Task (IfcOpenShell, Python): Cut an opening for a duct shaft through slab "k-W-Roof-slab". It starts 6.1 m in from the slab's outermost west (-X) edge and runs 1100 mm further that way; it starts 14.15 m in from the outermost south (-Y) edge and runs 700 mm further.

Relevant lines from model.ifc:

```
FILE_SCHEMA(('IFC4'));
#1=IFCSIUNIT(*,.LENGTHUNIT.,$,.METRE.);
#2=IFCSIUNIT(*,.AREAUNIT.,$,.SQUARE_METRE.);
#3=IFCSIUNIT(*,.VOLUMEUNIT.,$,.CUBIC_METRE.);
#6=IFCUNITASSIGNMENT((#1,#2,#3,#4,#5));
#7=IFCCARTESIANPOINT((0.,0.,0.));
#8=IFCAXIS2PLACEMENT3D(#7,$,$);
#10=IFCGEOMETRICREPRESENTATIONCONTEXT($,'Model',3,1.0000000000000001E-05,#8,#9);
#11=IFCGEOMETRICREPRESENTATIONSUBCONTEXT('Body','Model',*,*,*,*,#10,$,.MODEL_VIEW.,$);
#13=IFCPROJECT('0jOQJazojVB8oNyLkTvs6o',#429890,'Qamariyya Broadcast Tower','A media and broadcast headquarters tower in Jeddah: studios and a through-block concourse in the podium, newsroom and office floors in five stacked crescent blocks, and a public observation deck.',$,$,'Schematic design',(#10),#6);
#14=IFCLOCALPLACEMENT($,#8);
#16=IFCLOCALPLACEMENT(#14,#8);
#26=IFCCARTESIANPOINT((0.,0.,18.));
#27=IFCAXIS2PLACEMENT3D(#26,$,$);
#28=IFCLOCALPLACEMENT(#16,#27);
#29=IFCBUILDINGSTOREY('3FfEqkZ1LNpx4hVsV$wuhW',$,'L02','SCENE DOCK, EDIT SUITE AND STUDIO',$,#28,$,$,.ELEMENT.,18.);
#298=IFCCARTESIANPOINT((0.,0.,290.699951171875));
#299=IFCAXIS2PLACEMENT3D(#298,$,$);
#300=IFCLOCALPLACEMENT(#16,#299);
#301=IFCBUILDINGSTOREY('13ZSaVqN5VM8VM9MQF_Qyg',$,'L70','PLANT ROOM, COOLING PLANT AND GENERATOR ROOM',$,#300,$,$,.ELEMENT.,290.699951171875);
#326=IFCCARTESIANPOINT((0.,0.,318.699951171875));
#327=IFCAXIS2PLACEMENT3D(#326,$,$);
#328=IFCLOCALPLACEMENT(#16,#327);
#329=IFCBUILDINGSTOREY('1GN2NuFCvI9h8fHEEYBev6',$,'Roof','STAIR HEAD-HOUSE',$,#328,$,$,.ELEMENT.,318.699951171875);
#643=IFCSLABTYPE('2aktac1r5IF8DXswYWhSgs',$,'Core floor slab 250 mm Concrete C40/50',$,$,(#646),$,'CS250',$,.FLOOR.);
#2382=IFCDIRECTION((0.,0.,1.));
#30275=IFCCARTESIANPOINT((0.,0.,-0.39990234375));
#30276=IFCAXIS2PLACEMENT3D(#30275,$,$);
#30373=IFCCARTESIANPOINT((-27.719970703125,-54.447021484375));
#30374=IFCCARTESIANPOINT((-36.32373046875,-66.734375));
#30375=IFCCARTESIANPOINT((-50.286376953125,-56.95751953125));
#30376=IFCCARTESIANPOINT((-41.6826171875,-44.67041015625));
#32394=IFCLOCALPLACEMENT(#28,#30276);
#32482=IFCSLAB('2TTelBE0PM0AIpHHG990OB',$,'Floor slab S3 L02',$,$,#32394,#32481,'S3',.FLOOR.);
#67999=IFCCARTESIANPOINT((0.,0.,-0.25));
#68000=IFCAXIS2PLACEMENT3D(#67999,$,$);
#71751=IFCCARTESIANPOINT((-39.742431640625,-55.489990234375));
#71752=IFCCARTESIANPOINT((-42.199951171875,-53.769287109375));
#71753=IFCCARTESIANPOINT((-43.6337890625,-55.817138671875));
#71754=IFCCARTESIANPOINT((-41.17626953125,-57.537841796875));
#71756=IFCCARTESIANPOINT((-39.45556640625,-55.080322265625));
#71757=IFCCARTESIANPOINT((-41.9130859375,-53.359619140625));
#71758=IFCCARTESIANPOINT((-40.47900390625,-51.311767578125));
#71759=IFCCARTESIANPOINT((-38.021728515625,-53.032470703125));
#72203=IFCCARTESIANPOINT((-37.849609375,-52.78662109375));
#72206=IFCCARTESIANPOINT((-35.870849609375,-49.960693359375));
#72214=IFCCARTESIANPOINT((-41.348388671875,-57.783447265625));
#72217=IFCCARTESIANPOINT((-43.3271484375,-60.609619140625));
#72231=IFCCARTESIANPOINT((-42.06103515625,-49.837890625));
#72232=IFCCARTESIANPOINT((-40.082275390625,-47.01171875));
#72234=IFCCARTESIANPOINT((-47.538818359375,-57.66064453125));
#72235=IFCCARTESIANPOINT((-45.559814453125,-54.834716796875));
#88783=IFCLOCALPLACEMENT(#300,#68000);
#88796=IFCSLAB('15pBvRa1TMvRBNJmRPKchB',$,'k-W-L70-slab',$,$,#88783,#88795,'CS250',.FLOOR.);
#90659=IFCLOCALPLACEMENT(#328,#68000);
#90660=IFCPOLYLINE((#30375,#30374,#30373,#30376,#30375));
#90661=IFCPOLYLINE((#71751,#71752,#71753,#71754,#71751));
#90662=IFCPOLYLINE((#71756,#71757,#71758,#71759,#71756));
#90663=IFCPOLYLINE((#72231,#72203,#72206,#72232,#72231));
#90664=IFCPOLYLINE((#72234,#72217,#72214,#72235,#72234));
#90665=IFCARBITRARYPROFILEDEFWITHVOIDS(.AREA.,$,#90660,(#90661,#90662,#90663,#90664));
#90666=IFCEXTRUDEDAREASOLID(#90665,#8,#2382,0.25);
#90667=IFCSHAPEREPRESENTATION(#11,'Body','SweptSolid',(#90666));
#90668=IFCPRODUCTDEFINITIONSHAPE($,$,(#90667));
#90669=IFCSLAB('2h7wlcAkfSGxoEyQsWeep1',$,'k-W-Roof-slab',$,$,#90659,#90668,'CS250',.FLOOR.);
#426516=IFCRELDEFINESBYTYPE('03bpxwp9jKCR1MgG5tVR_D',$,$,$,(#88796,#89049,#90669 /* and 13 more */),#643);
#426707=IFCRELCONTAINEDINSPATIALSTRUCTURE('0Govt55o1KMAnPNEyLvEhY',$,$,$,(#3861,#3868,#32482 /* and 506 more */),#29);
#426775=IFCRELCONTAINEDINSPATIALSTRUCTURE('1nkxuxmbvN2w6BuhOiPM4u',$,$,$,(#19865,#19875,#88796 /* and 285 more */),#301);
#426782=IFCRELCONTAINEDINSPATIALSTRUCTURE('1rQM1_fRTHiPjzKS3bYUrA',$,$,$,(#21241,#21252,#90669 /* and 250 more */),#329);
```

```python
import numpy as np
import ifcopenshell
import ifcopenshell.api.feature
import ifcopenshell.api.geometry
import ifcopenshell.api.root
import ifcopenshell.geom
import ifcopenshell.util.placement
import ifcopenshell.util.representation
import ifcopenshell.util.shape
import ifcopenshell.util.unit

model = ifcopenshell.open("model.ifc")
unit_scale = ifcopenshell.util.unit.calculate_unit_scale(model)
settings = ifcopenshell.geom.settings()


def volume(element):
    """Net volume in cubic metres, openings subtracted."""
    shape = ifcopenshell.geom.create_shape(settings, element)
    return ifcopenshell.util.shape.get_volume(shape.geometry)


slab = model.by_guid("2h7wlcAkfSGxoEyQsWeep1")
before = volume(slab)

# Extent in the slab's own axes, in metres. The edges named are its -X and -Y sides.
slab_shape = ifcopenshell.geom.create_shape(settings, slab)
vertices = ifcopenshell.util.shape.get_vertices(slab_shape.geometry)
x_min, y_min, bottom = vertices.min(axis=0)
top = vertices[:, 2].max()

opening = ifcopenshell.api.root.create_entity(model, ifc_class="IfcOpeningElement", name="Duct shaft opening", predefined_type="OPENING")
context = ifcopenshell.util.representation.get_context(model, "Model", "Body", "MODEL_VIEW")
width, depth = 1.1, 0.7
outline = [(0.0, 0.0), (width, 0.0), (width, depth), (0.0, depth), (0.0, 0.0)]
# Overshoot both faces by 50 mm so the cut is clean.
shape = ifcopenshell.api.geometry.add_slab_representation(
    model, context=context, depth=top - bottom + 0.1, polyline=outline
)
ifcopenshell.api.geometry.assign_representation(model, product=opening, representation=shape)

matrix = ifcopenshell.util.placement.get_local_placement(slab.ObjectPlacement)
matrix[:, 3] = matrix @ np.append(np.array([x_min + 6.1, y_min + 14.15, bottom - 0.05]) / unit_scale, 1.0)
ifcopenshell.api.geometry.edit_object_placement(model, product=opening, matrix=matrix, is_si=False)
ifcopenshell.api.feature.add_feature(model, feature=opening, element=slab)

after = volume(slab)

print(f"slab volume {before:.3f} -> {after:.3f} m3")

model.write("model_edited.ifc")
```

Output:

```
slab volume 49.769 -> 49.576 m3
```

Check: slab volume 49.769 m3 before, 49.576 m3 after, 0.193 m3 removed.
